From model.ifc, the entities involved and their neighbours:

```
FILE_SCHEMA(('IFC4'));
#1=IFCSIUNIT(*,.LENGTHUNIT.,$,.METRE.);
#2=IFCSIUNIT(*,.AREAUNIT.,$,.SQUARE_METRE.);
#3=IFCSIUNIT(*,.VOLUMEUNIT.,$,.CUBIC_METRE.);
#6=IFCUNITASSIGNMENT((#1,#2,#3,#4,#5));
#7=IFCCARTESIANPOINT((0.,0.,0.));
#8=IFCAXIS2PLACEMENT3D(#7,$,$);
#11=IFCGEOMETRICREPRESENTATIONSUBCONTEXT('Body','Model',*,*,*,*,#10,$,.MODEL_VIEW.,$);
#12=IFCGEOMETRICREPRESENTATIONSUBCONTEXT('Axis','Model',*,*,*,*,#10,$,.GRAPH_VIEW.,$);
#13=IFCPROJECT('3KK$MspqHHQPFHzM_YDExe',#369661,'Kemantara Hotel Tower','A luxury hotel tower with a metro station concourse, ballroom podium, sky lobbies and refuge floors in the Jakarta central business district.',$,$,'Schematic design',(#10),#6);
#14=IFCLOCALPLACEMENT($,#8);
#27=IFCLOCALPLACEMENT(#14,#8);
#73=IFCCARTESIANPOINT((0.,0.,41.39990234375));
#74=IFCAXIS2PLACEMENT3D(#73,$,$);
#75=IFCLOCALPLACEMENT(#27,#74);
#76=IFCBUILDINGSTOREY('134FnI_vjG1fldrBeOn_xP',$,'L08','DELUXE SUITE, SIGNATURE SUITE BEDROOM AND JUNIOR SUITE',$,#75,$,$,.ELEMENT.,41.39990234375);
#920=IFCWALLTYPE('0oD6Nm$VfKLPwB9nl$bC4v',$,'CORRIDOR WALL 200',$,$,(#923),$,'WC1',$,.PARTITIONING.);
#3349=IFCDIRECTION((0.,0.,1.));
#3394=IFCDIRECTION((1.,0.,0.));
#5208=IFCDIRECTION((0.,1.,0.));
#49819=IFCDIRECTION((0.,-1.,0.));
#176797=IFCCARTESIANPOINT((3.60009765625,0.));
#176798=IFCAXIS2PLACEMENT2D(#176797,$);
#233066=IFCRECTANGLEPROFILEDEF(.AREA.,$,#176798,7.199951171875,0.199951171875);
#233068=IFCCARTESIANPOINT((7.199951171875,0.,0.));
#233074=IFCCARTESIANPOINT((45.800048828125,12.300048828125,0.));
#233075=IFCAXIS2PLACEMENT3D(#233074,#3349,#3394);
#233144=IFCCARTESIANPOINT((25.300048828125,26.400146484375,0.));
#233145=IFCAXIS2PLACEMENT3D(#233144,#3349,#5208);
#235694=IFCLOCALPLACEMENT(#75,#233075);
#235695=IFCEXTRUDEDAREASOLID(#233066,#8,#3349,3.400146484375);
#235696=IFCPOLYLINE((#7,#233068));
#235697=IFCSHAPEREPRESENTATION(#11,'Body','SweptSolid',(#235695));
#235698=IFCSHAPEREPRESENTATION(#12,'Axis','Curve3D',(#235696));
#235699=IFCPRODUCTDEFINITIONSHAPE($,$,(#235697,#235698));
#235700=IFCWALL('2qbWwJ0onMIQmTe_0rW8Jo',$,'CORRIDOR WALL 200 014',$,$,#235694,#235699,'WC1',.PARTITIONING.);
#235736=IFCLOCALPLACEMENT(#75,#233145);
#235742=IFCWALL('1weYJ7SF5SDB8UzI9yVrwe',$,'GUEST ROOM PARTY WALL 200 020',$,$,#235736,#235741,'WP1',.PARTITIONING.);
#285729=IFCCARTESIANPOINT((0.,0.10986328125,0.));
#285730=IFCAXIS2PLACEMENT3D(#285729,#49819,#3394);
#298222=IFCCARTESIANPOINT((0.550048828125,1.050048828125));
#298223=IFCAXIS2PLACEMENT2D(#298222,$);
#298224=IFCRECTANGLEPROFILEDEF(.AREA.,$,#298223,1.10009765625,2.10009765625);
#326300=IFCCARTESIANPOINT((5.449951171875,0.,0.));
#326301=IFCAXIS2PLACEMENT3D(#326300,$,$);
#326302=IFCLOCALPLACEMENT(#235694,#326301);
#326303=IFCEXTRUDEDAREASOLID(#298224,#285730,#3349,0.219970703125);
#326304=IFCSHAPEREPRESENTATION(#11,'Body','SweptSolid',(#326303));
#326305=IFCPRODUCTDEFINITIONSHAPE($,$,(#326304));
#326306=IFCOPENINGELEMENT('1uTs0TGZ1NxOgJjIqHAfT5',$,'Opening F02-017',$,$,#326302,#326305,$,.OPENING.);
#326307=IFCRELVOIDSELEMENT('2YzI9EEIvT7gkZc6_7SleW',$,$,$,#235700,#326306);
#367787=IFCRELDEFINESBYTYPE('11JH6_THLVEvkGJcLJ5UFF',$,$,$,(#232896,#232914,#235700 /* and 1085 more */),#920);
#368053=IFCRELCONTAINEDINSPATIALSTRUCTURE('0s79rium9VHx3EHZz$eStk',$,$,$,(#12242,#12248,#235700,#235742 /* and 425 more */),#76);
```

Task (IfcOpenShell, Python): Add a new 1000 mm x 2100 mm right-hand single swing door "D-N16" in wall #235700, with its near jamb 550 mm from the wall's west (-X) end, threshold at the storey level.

```python
import numpy as np
import ifcopenshell
import ifcopenshell.api.feature
import ifcopenshell.api.geometry
import ifcopenshell.api.root
import ifcopenshell.api.spatial
import ifcopenshell.geom
import ifcopenshell.util.element
import ifcopenshell.util.placement
import ifcopenshell.util.representation
import ifcopenshell.util.shape
import ifcopenshell.util.unit

model = ifcopenshell.open("model.ifc")
unit_scale = ifcopenshell.util.unit.calculate_unit_scale(model)
settings = ifcopenshell.geom.settings()


def volume(element):
    """Net volume in cubic metres, openings subtracted."""
    shape = ifcopenshell.geom.create_shape(settings, element)
    return ifcopenshell.util.shape.get_volume(shape.geometry)


wall = model.by_guid("2qbWwJ0onMIQmTe_0rW8Jo")
storey = ifcopenshell.util.element.get_container(wall, ifc_class="IfcBuildingStorey")
context = ifcopenshell.util.representation.get_context(model, "Model", "Body", "MODEL_VIEW")
before = volume(wall)

width, height, from_end, sill = 1, 2.1, 0.55, 0.0  # metres

# The wall runs along its own X axis, and the end named is its -X end.
wall_shape = ifcopenshell.geom.create_shape(settings, wall)
x, y, z = ifcopenshell.util.shape.get_vertices(wall_shape.geometry).T
start = x.min() + from_end
face, thickness = float(y.min()), float(y.max() - y.min())
wall_matrix = ifcopenshell.util.placement.get_local_placement(wall.ObjectPlacement)
level = ifcopenshell.util.placement.get_local_placement(storey.ObjectPlacement)[2, 3]


def in_wall(x, y):
    """Placement at x, y metres in the wall's axes, at sill height."""
    matrix = wall_matrix.copy()
    matrix[:, 3] = wall_matrix @ np.array([x / unit_scale, y / unit_scale, 0.0, 1.0])
    matrix[2, 3] = level + sill / unit_scale
    return matrix


# Opening: a box that overshoots both wall faces by 50 mm.
opening = ifcopenshell.api.root.create_entity(model, ifc_class="IfcOpeningElement", predefined_type="OPENING")
box = ifcopenshell.api.geometry.add_wall_representation(
    model, context=context, length=width, height=height, thickness=thickness + 0.1
)
ifcopenshell.api.geometry.assign_representation(model, product=opening, representation=box)
ifcopenshell.api.geometry.edit_object_placement(model, product=opening, matrix=in_wall(start, face - 0.05), is_si=False)
ifcopenshell.api.feature.add_feature(model, feature=opening, element=wall)

door = ifcopenshell.api.root.create_entity(model, ifc_class="IfcDoor", name="D-N16", predefined_type="DOOR")
door.OverallWidth, door.OverallHeight = width / unit_scale, height / unit_scale
door.OperationType = "SINGLE_SWING_RIGHT"
body = ifcopenshell.api.geometry.add_door_representation(
    model,
    context=context,
    overall_width=door.OverallWidth,
    overall_height=door.OverallHeight,
    operation_type="SINGLE_SWING_RIGHT",
    lining_properties={"LiningDepth": thickness / unit_scale, "ThresholdDepth": thickness / unit_scale},
)
ifcopenshell.api.geometry.assign_representation(model, product=door, representation=body)
ifcopenshell.api.spatial.assign_container(model, products=[door], relating_structure=storey)
ifcopenshell.api.feature.add_filling(model, opening=opening, element=door)

# The lining spans the wall, so the door starts at the wall face.
ifcopenshell.api.geometry.edit_object_placement(model, product=door, matrix=in_wall(start, face), is_si=False)

after = volume(wall)

print(f"wall volume {before:.3f} -> {after:.3f} m3")

model.write("model_v2.ifc")
```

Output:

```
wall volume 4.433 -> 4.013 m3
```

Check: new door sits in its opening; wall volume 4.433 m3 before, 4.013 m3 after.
